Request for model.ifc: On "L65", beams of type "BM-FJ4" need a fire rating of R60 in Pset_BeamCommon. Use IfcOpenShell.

First a look at what the model holds.

```python
import ifcopenshell
import ifcopenshell.util.element

model = ifcopenshell.open("model.ifc")
print(model.schema)
storey = next(s for s in model.by_type("IfcBuildingStorey") if s.Name == "L65")
beams = [e for e in ifcopenshell.util.element.get_decomposition(storey) if e.is_a("IfcBeam")]
seen = {}
for e in beams:
    element_type = ifcopenshell.util.element.get_type(e)
    key = (element_type.Name if element_type != e and element_type else None, ifcopenshell.util.element.get_pset(e, "Pset_BeamCommon", "FireRating"))
    seen[key] = seen.get(key, 0) + 1
for (name, value), count in sorted(seen.items(), key=str):
    print(count, "x", name, "|", value)
```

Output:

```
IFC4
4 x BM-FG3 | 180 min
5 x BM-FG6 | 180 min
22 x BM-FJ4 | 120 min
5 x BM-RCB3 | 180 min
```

```python
import ifcopenshell
import ifcopenshell.api.pset
import ifcopenshell.util.element

model = ifcopenshell.open("model.ifc")

storey = next(s for s in model.by_type("IfcBuildingStorey") if s.Name == "L65")
beams = [e for e in ifcopenshell.util.element.get_decomposition(storey) if e.is_a("IfcBeam")]

count = 0
for e in beams:
    element_type = ifcopenshell.util.element.get_type(e)
    if element_type in (None, e) or element_type.Name != "BM-FJ4":
        continue
    found = ifcopenshell.util.element.get_pset(e, "Pset_BeamCommon", should_inherit=False)
    if found:
        pset = model.by_id(found["id"])
        if len(ifcopenshell.util.element.get_elements_by_pset(pset)) > 1:
            pset = ifcopenshell.api.pset.unshare_pset(model, products=[e], pset=pset)[0]
    else:
        pset = ifcopenshell.api.pset.add_pset(model, product=e, name="Pset_BeamCommon")
    ifcopenshell.api.pset.edit_pset(model, pset=pset, properties={"FireRating": "R60"})
    count += 1

print(count, "beams updated")

model.write("model_updated.ifc")
```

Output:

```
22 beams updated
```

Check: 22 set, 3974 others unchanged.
